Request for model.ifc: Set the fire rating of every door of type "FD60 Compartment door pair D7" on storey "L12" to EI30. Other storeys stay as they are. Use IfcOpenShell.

First a look at what the model holds.

```python
import ifcopenshell
import ifcopenshell.util.element

model = ifcopenshell.open("model.ifc")
print(model.schema)
storey = next(s for s in model.by_type("IfcBuildingStorey") if s.Name == "L12")
doors = [e for e in ifcopenshell.util.element.get_decomposition(storey) if e.is_a("IfcDoor")]
seen = {}
for e in doors:
    element_type = ifcopenshell.util.element.get_type(e)
    key = (element_type.Name if element_type != e and element_type else None, ifcopenshell.util.element.get_pset(e, "Pset_DoorCommon", "FireRating"))
    seen[key] = seen.get(key, 0) + 1
for (name, value), count in sorted(seen.items(), key=str):
    print(count, "x", name, "|", value)
```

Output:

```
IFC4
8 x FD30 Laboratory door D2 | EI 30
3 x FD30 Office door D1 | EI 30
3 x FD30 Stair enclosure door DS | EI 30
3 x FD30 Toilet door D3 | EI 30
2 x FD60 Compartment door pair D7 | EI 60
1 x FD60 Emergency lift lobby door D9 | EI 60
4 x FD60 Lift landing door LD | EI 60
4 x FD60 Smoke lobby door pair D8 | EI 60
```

```python
import ifcopenshell
import ifcopenshell.api.pset
import ifcopenshell.util.element

model = ifcopenshell.open("model.ifc")

storey = next(s for s in model.by_type("IfcBuildingStorey") if s.Name == "L12")
doors = [e for e in ifcopenshell.util.element.get_decomposition(storey) if e.is_a("IfcDoor")]

count = 0
for e in doors:
    element_type = ifcopenshell.util.element.get_type(e)
    if element_type in (None, e) or element_type.Name != "FD60 Compartment door pair D7":
        continue
    # add_pset returns the element's existing set when there is one.
    pset = ifcopenshell.api.pset.add_pset(model, product=e, name="Pset_DoorCommon")
    ifcopenshell.api.pset.edit_pset(model, pset=pset, properties={"FireRating": "EI30"})
    count += 1

print(count, "doors updated")

model.write("model_edited.ifc")
```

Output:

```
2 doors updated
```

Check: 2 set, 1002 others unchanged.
